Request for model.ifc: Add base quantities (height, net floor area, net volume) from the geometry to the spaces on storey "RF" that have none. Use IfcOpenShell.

First a look at what the model holds.

```python
import ifcopenshell
import ifcopenshell.util.element
import ifcopenshell.util.unit

model = ifcopenshell.open("model.ifc")
print(model.schema)
for unit_type in ("LENGTHUNIT", "AREAUNIT", "VOLUMEUNIT"):
    print(unit_type, ifcopenshell.util.unit.calculate_unit_scale(model, unit_type))
storey = next(s for s in model.by_type("IfcBuildingStorey") if s.Name == "RF")
spaces = [e for e in ifcopenshell.util.element.get_decomposition(storey) if e.is_a("IfcSpace")]
for e in sorted(spaces, key=lambda e: e.id()):
    print(e.id(), e.is_a(), e.Name, list(ifcopenshell.util.element.get_psets(e, qtos_only=True)), sep=" | ")
```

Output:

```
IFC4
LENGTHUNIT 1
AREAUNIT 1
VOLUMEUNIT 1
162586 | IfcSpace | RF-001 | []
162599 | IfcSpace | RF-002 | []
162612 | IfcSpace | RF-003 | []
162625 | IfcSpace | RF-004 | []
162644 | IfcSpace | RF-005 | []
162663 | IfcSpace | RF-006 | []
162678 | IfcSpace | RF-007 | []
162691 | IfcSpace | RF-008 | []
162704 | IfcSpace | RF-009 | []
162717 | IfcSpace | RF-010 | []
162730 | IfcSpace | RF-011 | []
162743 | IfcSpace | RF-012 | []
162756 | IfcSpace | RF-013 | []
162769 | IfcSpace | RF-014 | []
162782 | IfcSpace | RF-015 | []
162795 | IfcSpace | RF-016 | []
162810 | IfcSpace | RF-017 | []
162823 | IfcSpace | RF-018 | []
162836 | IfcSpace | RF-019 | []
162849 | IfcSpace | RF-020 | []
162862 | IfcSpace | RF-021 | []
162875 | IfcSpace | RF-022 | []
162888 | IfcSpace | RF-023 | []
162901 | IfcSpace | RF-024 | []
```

```python
import ifcopenshell
import ifcopenshell.api.pset
import ifcopenshell.geom
import ifcopenshell.util.element
import ifcopenshell.util.shape
import ifcopenshell.util.unit

model = ifcopenshell.open("model.ifc")
unit_scale = ifcopenshell.util.unit.calculate_unit_scale(model)
area_scale = ifcopenshell.util.unit.calculate_unit_scale(model, "AREAUNIT")
volume_scale = ifcopenshell.util.unit.calculate_unit_scale(model, "VOLUMEUNIT")
settings = ifcopenshell.geom.settings()

storey = next(s for s in model.by_type("IfcBuildingStorey") if s.Name == "RF")
spaces = [e for e in ifcopenshell.util.element.get_decomposition(storey) if e.is_a("IfcSpace")]

for e in sorted(spaces, key=lambda e: e.id()):
    if ifcopenshell.util.element.get_psets(e, qtos_only=True, should_inherit=False):
        continue
    # Geometry comes back in metres, in the element's own axes.
    shape = ifcopenshell.geom.create_shape(settings, e)
    values = {
        "Height": ifcopenshell.util.shape.get_z(shape.geometry) / unit_scale,
        "NetFloorArea": ifcopenshell.util.shape.get_footprint_area(shape.geometry) / area_scale,
        "NetVolume": ifcopenshell.util.shape.get_volume(shape.geometry) / volume_scale,
    }
    qto = ifcopenshell.api.pset.add_qto(model, product=e, name="Qto_SpaceBaseQuantities")
    ifcopenshell.api.pset.edit_qto(model, qto=qto, properties=values)
    print(e.id(), {k: round(v, 3) for k, v in values.items()})

model.write("model-out.ifc")
```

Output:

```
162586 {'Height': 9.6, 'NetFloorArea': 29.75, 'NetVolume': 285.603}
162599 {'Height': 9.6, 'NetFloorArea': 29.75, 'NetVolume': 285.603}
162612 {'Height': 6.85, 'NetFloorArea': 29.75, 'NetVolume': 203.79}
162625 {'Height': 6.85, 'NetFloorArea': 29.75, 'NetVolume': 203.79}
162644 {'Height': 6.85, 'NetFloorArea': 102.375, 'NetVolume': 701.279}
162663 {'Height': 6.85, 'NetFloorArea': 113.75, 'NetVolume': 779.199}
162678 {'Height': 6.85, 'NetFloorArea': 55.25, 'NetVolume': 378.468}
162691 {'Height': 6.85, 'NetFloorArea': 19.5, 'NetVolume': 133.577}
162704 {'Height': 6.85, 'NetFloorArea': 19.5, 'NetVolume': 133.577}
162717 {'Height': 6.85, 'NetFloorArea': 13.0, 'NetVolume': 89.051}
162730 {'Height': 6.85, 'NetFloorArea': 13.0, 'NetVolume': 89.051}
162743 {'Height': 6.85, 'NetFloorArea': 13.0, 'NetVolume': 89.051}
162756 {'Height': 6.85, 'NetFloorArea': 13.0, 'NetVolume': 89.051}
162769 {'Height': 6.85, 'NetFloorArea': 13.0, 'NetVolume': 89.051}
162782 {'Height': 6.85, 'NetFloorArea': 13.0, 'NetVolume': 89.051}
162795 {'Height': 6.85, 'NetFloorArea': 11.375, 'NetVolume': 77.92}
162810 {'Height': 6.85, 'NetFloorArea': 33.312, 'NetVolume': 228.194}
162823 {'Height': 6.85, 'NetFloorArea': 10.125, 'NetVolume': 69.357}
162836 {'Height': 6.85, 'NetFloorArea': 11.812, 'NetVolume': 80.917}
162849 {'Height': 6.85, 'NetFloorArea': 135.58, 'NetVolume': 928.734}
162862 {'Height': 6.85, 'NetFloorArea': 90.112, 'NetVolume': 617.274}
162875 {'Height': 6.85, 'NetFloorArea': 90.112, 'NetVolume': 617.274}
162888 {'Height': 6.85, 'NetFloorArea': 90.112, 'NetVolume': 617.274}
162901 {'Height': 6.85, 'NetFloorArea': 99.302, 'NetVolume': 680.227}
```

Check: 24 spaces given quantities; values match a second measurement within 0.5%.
